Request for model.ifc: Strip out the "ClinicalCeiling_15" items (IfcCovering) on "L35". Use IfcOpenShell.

First a look at what the model holds.

```python
import ifcopenshell
import ifcopenshell.util.element

model = ifcopenshell.open("model.ifc")
print(model.schema)
storey = next(s for s in model.by_type("IfcBuildingStorey") if s.Name == "L35")
coverings = [e for e in ifcopenshell.util.element.get_decomposition(storey) if e.is_a("IfcCovering")]
seen = {}
for e in coverings:
    element_type = ifcopenshell.util.element.get_type(e)
    name = element_type.Name if element_type not in (None, e) else None
    seen[name] = seen.get(name, 0) + 1
for name, count in sorted(seen.items(), key=str):
    print(count, "x", name)
```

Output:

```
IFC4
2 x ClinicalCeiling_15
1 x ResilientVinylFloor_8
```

```python
import ifcopenshell
import ifcopenshell.api.root
import ifcopenshell.util.element

model = ifcopenshell.open("model.ifc")

storey = next(s for s in model.by_type("IfcBuildingStorey") if s.Name == "L35")
coverings = [e for e in ifcopenshell.util.element.get_decomposition(storey) if e.is_a("IfcCovering")]
targets = [e for e in coverings if (t := ifcopenshell.util.element.get_type(e)) not in (None, e) and t.Name == "ClinicalCeiling_15"]

for e in targets:
    ifcopenshell.api.root.remove_product(model, product=e)
print(len(targets), "removed")

model.write("model_edited.ifc")
```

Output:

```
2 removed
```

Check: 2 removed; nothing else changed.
